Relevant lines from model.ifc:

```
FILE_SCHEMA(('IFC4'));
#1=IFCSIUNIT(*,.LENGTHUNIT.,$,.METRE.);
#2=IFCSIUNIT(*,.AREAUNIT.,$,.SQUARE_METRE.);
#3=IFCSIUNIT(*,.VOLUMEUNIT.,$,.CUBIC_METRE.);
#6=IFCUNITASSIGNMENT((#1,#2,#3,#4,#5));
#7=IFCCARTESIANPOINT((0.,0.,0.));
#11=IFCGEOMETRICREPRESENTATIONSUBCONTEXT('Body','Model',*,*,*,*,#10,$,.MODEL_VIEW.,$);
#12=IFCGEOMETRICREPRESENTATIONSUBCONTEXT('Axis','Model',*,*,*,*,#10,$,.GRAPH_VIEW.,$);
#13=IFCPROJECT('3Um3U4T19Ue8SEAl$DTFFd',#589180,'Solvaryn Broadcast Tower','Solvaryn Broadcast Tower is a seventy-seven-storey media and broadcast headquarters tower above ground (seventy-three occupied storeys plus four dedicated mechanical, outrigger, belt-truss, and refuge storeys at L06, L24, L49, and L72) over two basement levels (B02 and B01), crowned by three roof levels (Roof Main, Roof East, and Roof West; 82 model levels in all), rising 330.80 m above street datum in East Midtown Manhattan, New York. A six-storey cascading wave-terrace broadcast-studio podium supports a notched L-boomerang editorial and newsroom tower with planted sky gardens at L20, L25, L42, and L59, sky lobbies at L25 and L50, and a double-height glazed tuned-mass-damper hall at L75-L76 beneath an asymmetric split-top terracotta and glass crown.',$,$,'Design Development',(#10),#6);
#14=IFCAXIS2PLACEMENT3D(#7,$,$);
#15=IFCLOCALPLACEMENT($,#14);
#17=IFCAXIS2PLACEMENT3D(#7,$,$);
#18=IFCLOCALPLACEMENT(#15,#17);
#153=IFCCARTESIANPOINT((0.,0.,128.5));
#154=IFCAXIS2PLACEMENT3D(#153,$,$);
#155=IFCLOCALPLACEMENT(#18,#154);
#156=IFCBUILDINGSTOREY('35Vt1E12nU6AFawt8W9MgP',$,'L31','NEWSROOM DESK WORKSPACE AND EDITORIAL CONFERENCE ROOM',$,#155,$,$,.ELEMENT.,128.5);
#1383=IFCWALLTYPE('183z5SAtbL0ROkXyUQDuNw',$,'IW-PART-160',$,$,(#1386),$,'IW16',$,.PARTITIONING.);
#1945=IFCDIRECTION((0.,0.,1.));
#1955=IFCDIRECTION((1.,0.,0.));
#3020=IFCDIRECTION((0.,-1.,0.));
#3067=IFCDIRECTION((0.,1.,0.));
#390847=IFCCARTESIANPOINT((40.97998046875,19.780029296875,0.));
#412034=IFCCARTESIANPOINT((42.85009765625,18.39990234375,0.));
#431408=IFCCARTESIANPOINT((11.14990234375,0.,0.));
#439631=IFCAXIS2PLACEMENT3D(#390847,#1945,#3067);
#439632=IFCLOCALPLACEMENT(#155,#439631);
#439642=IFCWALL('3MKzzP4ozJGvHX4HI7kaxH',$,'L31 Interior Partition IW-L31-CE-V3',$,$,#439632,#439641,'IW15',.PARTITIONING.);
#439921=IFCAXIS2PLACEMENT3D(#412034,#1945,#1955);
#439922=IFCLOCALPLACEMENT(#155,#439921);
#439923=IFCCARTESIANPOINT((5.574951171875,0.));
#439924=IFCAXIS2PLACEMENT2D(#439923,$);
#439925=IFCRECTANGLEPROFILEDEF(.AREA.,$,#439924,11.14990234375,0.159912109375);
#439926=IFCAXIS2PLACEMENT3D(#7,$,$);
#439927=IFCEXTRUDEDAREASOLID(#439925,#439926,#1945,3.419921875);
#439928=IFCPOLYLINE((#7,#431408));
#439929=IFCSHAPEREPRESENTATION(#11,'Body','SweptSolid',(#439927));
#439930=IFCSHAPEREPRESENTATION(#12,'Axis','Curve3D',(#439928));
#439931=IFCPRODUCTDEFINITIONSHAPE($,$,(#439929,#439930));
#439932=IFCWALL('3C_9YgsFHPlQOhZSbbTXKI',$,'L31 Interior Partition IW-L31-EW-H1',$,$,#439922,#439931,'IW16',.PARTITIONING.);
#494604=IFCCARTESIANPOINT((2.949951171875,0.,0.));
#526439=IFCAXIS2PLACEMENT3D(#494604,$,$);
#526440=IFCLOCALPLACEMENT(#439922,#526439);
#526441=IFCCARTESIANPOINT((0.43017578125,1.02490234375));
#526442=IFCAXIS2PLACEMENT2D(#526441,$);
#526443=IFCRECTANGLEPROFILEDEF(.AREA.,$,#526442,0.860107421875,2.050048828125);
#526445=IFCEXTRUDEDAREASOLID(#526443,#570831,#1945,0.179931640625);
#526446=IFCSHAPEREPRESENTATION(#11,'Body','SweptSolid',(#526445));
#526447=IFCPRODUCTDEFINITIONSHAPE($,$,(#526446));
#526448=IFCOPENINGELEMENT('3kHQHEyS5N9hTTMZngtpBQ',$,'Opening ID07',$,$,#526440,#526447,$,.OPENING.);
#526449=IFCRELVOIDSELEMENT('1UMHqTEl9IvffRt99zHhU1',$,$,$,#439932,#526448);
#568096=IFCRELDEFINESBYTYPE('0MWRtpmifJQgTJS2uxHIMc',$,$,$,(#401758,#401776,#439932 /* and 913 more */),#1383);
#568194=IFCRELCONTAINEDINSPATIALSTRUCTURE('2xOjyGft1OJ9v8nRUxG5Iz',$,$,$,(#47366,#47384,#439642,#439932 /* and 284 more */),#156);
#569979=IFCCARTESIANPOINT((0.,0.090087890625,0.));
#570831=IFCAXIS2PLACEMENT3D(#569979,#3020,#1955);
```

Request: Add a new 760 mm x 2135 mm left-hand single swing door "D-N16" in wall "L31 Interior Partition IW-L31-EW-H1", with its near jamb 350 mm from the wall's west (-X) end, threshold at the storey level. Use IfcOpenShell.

```python
import numpy as np
import ifcopenshell
import ifcopenshell.api.feature
import ifcopenshell.api.geometry
import ifcopenshell.api.root
import ifcopenshell.api.spatial
import ifcopenshell.geom
import ifcopenshell.util.element
import ifcopenshell.util.placement
import ifcopenshell.util.representation
import ifcopenshell.util.shape
import ifcopenshell.util.unit

model = ifcopenshell.open("model.ifc")
unit_scale = ifcopenshell.util.unit.calculate_unit_scale(model)
settings = ifcopenshell.geom.settings()


def volume(element):
    """Net volume in cubic metres, openings subtracted."""
    shape = ifcopenshell.geom.create_shape(settings, element)
    return ifcopenshell.util.shape.get_volume(shape.geometry)


wall = model.by_guid("3C_9YgsFHPlQOhZSbbTXKI")
storey = ifcopenshell.util.element.get_container(wall, ifc_class="IfcBuildingStorey")
context = ifcopenshell.util.representation.get_context(model, "Model", "Body", "MODEL_VIEW")
before = volume(wall)

width, height, from_end, sill = 0.76, 2.135, 0.35, 0.0  # metres

# The wall runs along its own X axis, and the end named is its -X end.
wall_shape = ifcopenshell.geom.create_shape(settings, wall)
x, y, z = ifcopenshell.util.shape.get_vertices(wall_shape.geometry).T
start = x.min() + from_end
face, thickness = float(y.min()), float(y.max() - y.min())
wall_matrix = ifcopenshell.util.placement.get_local_placement(wall.ObjectPlacement)
level = ifcopenshell.util.placement.get_local_placement(storey.ObjectPlacement)[2, 3]


def in_wall(x, y):
    """Placement at x, y metres in the wall's axes, at sill height."""
    matrix = wall_matrix.copy()
    matrix[:, 3] = wall_matrix @ np.array([x / unit_scale, y / unit_scale, 0.0, 1.0])
    matrix[2, 3] = level + sill / unit_scale
    return matrix


# Opening: a box that overshoots both wall faces by 50 mm.
opening = ifcopenshell.api.root.create_entity(model, ifc_class="IfcOpeningElement", predefined_type="OPENING")
box = ifcopenshell.api.geometry.add_wall_representation(
    model, context=context, length=width, height=height, thickness=thickness + 0.1
)
ifcopenshell.api.geometry.assign_representation(model, product=opening, representation=box)
ifcopenshell.api.geometry.edit_object_placement(model, product=opening, matrix=in_wall(start, face - 0.05), is_si=False)
ifcopenshell.api.feature.add_feature(model, feature=opening, element=wall)

door = ifcopenshell.api.root.create_entity(model, ifc_class="IfcDoor", name="D-N16", predefined_type="DOOR")
door.OverallWidth, door.OverallHeight = width / unit_scale, height / unit_scale
door.OperationType = "SINGLE_SWING_LEFT"
body = ifcopenshell.api.geometry.add_door_representation(
    model,
    context=context,
    overall_width=door.OverallWidth,
    overall_height=door.OverallHeight,
    operation_type="SINGLE_SWING_LEFT",
    lining_properties={"LiningDepth": thickness / unit_scale, "ThresholdDepth": thickness / unit_scale},
)
ifcopenshell.api.geometry.assign_representation(model, product=door, representation=body)
ifcopenshell.api.spatial.assign_container(model, products=[door], relating_structure=storey)
ifcopenshell.api.feature.add_filling(model, opening=opening, element=door)

# The lining spans the wall, so the door starts at the wall face.
ifcopenshell.api.geometry.edit_object_placement(model, product=door, matrix=in_wall(start, face), is_si=False)

after = volume(wall)

print(f"wall volume {before:.3f} -> {after:.3f} m3")

model.write("model_rev.ifc")
```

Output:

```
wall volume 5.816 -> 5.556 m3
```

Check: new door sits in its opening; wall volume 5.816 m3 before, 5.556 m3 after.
